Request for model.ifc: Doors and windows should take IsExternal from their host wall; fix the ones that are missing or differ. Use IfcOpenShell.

First a look at what the model holds.

```python
import ifcopenshell
import ifcopenshell.util.element

model = ifcopenshell.open("model.ifc")
print(model.schema)
seen = {}
for e in model.by_type("IfcDoor") + model.by_type("IfcWindow"):
    if not e.FillsVoids:
        continue
    host = e.FillsVoids[0].RelatingOpeningElement.VoidsElements[0].RelatingBuildingElement
    own = ifcopenshell.util.element.get_pset(e, f"Pset_{e.is_a()[3:].removesuffix('StandardCase')}Common", "IsExternal")
    wall = ifcopenshell.util.element.get_pset(host, "Pset_WallCommon", "IsExternal")
    seen[e.is_a(), own, wall] = seen.get((e.is_a(), own, wall), 0) + 1
for (cls, own, wall), count in sorted(seen.items(), key=str):
    print(count, cls, "IsExternal:", own, "| host wall:", wall)
```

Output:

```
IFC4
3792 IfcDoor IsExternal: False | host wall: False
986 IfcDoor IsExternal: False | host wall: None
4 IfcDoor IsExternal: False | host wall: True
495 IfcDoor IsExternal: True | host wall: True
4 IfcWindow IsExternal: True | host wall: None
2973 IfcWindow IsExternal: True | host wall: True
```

```python
import ifcopenshell
import ifcopenshell.api.pset
import ifcopenshell.util.element

model = ifcopenshell.open("model.ifc")

count = 0
for ifc_class, pset_name in (("IfcDoor", "Pset_DoorCommon"), ("IfcWindow", "Pset_WindowCommon")):
    for e in model.by_type(ifc_class):
        if not e.FillsVoids:
            continue
        host = e.FillsVoids[0].RelatingOpeningElement.VoidsElements[0].RelatingBuildingElement
        external = ifcopenshell.util.element.get_pset(host, "Pset_WallCommon", "IsExternal")
        if external is None or ifcopenshell.util.element.get_pset(e, pset_name, "IsExternal") == external:
            continue
        found = ifcopenshell.util.element.get_pset(e, pset_name, should_inherit=False)
        if found:
            pset = model.by_id(found["id"])
            if len(ifcopenshell.util.element.get_elements_by_pset(pset)) > 1:
                pset = ifcopenshell.api.pset.unshare_pset(model, products=[e], pset=pset)[0]
        else:
            pset = ifcopenshell.api.pset.add_pset(model, product=e, name=pset_name)
        ifcopenshell.api.pset.edit_pset(model, pset=pset, properties={"IsExternal": external})
        count += 1

print(count, "updated")

model.write("model_updated.ifc")
```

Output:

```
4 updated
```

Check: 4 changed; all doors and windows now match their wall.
